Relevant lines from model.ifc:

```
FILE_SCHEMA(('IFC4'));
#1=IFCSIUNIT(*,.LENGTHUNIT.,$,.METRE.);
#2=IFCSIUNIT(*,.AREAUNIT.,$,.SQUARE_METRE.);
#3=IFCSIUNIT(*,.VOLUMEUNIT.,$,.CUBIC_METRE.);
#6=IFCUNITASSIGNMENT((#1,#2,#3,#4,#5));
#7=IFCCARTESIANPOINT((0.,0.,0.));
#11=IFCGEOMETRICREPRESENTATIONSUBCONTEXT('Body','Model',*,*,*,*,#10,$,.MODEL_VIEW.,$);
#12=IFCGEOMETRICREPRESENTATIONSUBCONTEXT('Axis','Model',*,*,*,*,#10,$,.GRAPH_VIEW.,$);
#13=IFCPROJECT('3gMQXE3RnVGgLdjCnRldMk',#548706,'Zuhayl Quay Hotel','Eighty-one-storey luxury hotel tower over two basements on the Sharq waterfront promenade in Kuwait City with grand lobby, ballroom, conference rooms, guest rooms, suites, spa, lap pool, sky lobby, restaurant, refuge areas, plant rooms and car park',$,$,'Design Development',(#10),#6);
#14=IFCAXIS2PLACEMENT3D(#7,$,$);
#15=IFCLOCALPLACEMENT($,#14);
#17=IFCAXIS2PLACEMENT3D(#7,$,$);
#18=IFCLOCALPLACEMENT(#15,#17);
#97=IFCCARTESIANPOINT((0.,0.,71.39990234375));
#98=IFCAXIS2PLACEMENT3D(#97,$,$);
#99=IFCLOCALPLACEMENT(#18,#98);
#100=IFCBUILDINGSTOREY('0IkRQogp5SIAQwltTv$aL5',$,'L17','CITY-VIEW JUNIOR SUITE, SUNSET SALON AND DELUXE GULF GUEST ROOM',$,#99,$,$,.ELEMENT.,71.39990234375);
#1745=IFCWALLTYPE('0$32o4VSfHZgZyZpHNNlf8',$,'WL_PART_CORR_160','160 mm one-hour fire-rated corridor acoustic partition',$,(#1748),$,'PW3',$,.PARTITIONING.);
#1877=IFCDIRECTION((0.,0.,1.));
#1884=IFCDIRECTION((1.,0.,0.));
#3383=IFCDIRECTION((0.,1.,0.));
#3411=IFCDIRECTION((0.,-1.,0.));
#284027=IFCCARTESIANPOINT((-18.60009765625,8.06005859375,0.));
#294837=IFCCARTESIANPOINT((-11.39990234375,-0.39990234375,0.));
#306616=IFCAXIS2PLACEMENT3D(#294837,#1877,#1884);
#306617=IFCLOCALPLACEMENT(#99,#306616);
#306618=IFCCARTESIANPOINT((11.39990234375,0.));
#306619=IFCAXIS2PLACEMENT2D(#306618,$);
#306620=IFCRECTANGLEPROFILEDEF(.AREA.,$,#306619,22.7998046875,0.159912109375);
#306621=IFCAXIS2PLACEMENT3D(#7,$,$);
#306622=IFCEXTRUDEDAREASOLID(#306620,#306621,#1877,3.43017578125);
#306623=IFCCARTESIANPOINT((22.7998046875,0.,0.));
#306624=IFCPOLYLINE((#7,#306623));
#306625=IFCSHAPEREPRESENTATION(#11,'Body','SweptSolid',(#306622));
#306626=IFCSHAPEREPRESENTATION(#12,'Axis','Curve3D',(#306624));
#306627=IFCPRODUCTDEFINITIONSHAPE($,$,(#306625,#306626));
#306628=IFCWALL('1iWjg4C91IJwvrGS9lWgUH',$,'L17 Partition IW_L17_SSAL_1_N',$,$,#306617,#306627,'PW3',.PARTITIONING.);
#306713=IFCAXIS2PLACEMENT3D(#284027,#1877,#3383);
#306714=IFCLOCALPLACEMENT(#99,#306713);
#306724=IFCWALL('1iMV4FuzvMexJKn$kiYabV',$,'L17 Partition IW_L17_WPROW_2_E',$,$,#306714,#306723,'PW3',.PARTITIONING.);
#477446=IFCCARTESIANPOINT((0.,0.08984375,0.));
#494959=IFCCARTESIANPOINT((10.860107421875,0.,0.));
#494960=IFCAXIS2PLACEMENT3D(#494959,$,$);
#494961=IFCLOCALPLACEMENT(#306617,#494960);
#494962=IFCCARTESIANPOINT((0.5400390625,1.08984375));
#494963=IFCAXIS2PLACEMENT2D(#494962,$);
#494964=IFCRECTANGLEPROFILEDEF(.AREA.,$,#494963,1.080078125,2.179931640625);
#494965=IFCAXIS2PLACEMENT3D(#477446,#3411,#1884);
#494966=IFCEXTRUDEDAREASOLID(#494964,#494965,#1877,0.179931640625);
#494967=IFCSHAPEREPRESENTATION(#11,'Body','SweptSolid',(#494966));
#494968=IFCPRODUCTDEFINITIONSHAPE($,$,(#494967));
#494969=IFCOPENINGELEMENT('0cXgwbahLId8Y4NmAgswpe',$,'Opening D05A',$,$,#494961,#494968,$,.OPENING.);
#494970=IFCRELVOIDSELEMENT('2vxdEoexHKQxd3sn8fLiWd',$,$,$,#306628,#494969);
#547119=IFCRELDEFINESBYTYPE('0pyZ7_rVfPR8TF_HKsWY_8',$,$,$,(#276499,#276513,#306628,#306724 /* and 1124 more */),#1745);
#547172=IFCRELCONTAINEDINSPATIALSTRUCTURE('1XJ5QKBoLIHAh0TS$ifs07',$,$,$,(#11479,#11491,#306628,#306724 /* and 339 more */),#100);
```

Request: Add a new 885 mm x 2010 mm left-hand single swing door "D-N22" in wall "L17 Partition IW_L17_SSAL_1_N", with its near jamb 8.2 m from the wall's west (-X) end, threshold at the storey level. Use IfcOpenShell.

```python
import numpy as np
import ifcopenshell
import ifcopenshell.api.feature
import ifcopenshell.api.geometry
import ifcopenshell.api.root
import ifcopenshell.api.spatial
import ifcopenshell.geom
import ifcopenshell.util.element
import ifcopenshell.util.placement
import ifcopenshell.util.representation
import ifcopenshell.util.shape
import ifcopenshell.util.unit

model = ifcopenshell.open("model.ifc")
unit_scale = ifcopenshell.util.unit.calculate_unit_scale(model)
settings = ifcopenshell.geom.settings()


def volume(element):
    """Net volume in cubic metres, openings subtracted."""
    shape = ifcopenshell.geom.create_shape(settings, element)
    return ifcopenshell.util.shape.get_volume(shape.geometry)


wall = model.by_id(306628)
storey = ifcopenshell.util.element.get_container(wall, ifc_class="IfcBuildingStorey")
context = ifcopenshell.util.representation.get_context(model, "Model", "Body", "MODEL_VIEW")
before = volume(wall)

width, height, from_end, sill = 0.885, 2.01, 8.2, 0.0  # metres

# The wall runs along its own X axis, and the end named is its -X end.
wall_shape = ifcopenshell.geom.create_shape(settings, wall)
x, y, z = ifcopenshell.util.shape.get_vertices(wall_shape.geometry).T
start = x.min() + from_end
face, thickness = float(y.min()), float(y.max() - y.min())
wall_matrix = ifcopenshell.util.placement.get_local_placement(wall.ObjectPlacement)
level = ifcopenshell.util.placement.get_local_placement(storey.ObjectPlacement)[2, 3]


def in_wall(x, y):
    """Placement at x, y metres in the wall's axes, at sill height."""
    matrix = wall_matrix.copy()
    matrix[:, 3] = wall_matrix @ np.array([x / unit_scale, y / unit_scale, 0.0, 1.0])
    matrix[2, 3] = level + sill / unit_scale
    return matrix


# Opening: a box that overshoots both wall faces by 50 mm.
opening = ifcopenshell.api.root.create_entity(model, ifc_class="IfcOpeningElement", predefined_type="OPENING")
box = ifcopenshell.api.geometry.add_wall_representation(
    model, context=context, length=width, height=height, thickness=thickness + 0.1
)
ifcopenshell.api.geometry.assign_representation(model, product=opening, representation=box)
ifcopenshell.api.geometry.edit_object_placement(model, product=opening, matrix=in_wall(start, face - 0.05), is_si=False)
ifcopenshell.api.feature.add_feature(model, feature=opening, element=wall)

door = ifcopenshell.api.root.create_entity(model, ifc_class="IfcDoor", name="D-N22", predefined_type="DOOR")
door.OverallWidth, door.OverallHeight = width / unit_scale, height / unit_scale
door.OperationType = "SINGLE_SWING_LEFT"
body = ifcopenshell.api.geometry.add_door_representation(
    model,
    context=context,
    overall_width=door.OverallWidth,
    overall_height=door.OverallHeight,
    operation_type="SINGLE_SWING_LEFT",
    lining_properties={"LiningDepth": thickness / unit_scale, "ThresholdDepth": thickness / unit_scale},
)
ifcopenshell.api.geometry.assign_representation(model, product=door, representation=body)
ifcopenshell.api.spatial.assign_container(model, products=[door], relating_structure=storey)
ifcopenshell.api.feature.add_filling(model, opening=opening, element=door)

# The lining spans the wall, so the door starts at the wall face.
ifcopenshell.api.geometry.edit_object_placement(model, product=door, matrix=in_wall(start, face), is_si=False)

after = volume(wall)

print(f"wall volume {before:.3f} -> {after:.3f} m3")

model.write("model_v2.ifc")
```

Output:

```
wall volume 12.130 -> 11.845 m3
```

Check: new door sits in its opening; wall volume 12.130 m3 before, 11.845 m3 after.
